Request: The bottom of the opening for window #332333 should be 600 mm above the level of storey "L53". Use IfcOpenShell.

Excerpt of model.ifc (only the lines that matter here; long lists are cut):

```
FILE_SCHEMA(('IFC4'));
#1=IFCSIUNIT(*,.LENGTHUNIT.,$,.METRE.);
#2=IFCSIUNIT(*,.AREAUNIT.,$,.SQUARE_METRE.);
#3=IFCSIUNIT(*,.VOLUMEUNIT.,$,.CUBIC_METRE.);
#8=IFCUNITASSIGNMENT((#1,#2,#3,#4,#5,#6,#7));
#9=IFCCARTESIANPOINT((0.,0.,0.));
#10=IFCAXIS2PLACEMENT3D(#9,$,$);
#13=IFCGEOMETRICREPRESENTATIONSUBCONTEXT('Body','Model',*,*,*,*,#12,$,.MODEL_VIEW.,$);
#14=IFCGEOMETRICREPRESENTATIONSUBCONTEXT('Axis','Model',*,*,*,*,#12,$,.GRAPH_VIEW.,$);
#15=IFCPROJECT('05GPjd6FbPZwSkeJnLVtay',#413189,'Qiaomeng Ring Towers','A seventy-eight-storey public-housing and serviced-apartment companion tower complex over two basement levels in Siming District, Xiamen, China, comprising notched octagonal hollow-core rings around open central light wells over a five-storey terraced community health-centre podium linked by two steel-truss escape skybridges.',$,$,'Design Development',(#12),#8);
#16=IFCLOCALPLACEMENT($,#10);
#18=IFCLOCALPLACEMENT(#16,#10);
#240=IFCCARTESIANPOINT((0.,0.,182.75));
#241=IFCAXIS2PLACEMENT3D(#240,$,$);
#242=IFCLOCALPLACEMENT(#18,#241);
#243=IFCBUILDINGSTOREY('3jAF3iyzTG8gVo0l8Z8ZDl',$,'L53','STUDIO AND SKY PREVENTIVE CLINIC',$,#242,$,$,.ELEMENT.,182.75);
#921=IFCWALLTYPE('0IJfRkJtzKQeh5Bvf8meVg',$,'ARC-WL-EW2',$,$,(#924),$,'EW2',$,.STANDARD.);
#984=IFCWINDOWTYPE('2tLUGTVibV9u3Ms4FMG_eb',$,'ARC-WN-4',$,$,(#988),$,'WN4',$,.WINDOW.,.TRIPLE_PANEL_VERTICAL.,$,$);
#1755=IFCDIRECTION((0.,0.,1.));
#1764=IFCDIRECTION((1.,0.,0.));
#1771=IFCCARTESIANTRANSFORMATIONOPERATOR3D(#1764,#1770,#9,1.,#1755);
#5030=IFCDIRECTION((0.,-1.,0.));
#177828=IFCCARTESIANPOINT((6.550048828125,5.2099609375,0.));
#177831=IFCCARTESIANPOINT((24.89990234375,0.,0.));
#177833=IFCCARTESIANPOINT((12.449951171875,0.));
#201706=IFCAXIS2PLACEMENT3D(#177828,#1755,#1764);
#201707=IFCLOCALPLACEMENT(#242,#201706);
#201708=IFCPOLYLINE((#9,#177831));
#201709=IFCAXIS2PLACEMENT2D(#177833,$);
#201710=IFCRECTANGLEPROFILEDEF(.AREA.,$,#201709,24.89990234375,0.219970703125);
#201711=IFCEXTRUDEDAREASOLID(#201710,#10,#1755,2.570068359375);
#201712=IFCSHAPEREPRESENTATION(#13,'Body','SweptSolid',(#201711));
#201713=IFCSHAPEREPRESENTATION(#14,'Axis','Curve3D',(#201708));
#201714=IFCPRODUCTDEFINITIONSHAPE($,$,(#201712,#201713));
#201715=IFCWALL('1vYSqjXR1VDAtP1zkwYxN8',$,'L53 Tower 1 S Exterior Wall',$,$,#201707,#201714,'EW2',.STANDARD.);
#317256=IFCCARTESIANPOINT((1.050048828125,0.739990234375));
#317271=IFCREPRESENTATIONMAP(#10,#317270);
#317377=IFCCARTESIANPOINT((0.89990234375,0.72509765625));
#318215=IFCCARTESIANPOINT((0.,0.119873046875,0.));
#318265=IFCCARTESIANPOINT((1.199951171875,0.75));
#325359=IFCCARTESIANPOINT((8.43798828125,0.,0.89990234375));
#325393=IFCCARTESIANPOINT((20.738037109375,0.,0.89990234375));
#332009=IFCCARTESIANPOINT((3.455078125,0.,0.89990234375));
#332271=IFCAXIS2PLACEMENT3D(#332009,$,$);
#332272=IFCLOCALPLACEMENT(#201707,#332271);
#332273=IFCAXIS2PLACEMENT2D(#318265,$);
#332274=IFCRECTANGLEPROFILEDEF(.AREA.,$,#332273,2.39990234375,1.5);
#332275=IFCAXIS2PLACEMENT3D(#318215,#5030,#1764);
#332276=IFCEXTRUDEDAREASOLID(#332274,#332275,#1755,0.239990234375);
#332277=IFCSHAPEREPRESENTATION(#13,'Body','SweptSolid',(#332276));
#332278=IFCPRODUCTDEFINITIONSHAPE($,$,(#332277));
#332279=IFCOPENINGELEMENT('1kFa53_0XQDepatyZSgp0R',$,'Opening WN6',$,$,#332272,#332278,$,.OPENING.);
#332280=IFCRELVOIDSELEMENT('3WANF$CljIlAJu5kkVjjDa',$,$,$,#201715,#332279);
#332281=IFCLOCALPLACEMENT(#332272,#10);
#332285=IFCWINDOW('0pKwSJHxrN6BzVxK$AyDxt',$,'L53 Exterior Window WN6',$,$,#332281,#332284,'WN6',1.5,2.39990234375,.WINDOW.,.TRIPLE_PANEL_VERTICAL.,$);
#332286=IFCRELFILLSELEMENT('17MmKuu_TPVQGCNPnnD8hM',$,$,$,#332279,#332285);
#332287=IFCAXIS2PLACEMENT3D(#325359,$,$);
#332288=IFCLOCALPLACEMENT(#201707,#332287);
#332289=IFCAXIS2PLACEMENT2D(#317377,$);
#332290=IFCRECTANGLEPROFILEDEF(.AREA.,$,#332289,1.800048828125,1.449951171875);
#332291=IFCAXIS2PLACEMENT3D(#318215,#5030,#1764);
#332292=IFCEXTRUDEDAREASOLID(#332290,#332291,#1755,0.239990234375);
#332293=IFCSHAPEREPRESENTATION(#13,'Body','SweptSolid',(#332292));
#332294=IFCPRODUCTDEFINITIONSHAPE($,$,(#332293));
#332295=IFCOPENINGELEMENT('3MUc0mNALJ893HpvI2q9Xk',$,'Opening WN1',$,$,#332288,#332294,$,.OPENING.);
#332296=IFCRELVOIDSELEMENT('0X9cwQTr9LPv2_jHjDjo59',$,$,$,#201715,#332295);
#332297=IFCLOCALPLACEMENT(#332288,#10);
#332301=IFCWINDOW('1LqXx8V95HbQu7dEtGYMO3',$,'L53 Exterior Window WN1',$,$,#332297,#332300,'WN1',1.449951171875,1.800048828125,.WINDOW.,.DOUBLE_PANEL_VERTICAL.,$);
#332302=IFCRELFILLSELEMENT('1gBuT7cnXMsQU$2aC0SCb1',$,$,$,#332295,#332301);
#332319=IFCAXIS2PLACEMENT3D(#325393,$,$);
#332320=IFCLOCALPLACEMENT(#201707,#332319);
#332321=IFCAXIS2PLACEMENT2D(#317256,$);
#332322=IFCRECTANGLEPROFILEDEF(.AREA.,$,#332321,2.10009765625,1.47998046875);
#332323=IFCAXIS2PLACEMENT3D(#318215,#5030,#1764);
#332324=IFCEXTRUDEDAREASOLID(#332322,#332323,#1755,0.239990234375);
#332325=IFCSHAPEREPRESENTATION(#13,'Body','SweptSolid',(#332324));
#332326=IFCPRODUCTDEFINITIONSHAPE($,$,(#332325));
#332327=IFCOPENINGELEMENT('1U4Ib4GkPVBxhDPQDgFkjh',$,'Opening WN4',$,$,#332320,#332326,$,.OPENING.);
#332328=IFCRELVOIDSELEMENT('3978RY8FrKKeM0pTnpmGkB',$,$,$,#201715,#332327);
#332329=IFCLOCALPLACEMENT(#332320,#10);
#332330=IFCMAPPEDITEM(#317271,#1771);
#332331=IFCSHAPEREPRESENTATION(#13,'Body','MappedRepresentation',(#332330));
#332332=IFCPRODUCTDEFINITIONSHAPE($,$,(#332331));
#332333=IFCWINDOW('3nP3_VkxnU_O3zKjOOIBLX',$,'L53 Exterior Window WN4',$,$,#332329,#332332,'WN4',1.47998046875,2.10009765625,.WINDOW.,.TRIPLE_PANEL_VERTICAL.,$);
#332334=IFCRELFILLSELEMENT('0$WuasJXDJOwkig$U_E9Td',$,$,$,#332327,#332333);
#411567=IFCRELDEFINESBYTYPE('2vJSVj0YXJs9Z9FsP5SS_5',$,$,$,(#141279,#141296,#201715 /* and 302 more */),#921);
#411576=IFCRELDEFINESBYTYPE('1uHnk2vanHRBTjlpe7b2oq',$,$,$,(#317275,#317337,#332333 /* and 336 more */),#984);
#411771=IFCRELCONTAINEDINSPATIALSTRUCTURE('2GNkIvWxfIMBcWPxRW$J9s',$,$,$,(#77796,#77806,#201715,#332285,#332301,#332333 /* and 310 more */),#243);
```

```python
import numpy as np
import ifcopenshell
import ifcopenshell.api.geometry
import ifcopenshell.geom
import ifcopenshell.util.element
import ifcopenshell.util.placement
import ifcopenshell.util.shape
import ifcopenshell.util.unit

model = ifcopenshell.open("model.ifc")
unit_scale = ifcopenshell.util.unit.calculate_unit_scale(model)

window = model.by_guid("3nP3_VkxnU_O3zKjOOIBLX")
opening = window.FillsVoids[0].RelatingOpeningElement
storey = ifcopenshell.util.element.get_container(window, ifc_class="IfcBuildingStorey")
level = ifcopenshell.util.placement.get_local_placement(storey.ObjectPlacement)[2, 3]

# The opening's origin need not be at the sill, so measure its lowest point.
shape = ifcopenshell.geom.create_shape(ifcopenshell.geom.settings(), opening)
bottom = ifcopenshell.util.shape.get_shape_bottom_elevation(shape, shape.geometry) / unit_scale
dz = level + 0.6 / unit_scale - bottom

shift = np.array([0.0, 0.0, dz])
# The window is placed relative to its opening, so it follows when the opening moves.
matrix = ifcopenshell.util.placement.get_local_placement(opening.ObjectPlacement)
matrix[:3, 3] += shift
ifcopenshell.api.geometry.edit_object_placement(
    model, product=opening, matrix=matrix, is_si=False, should_transform_children=True
)

print(f"moved by {dz * unit_scale:+.3f} m")

model.write("model_updated.ifc")
```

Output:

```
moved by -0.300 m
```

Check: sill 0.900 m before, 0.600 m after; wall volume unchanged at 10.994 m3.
